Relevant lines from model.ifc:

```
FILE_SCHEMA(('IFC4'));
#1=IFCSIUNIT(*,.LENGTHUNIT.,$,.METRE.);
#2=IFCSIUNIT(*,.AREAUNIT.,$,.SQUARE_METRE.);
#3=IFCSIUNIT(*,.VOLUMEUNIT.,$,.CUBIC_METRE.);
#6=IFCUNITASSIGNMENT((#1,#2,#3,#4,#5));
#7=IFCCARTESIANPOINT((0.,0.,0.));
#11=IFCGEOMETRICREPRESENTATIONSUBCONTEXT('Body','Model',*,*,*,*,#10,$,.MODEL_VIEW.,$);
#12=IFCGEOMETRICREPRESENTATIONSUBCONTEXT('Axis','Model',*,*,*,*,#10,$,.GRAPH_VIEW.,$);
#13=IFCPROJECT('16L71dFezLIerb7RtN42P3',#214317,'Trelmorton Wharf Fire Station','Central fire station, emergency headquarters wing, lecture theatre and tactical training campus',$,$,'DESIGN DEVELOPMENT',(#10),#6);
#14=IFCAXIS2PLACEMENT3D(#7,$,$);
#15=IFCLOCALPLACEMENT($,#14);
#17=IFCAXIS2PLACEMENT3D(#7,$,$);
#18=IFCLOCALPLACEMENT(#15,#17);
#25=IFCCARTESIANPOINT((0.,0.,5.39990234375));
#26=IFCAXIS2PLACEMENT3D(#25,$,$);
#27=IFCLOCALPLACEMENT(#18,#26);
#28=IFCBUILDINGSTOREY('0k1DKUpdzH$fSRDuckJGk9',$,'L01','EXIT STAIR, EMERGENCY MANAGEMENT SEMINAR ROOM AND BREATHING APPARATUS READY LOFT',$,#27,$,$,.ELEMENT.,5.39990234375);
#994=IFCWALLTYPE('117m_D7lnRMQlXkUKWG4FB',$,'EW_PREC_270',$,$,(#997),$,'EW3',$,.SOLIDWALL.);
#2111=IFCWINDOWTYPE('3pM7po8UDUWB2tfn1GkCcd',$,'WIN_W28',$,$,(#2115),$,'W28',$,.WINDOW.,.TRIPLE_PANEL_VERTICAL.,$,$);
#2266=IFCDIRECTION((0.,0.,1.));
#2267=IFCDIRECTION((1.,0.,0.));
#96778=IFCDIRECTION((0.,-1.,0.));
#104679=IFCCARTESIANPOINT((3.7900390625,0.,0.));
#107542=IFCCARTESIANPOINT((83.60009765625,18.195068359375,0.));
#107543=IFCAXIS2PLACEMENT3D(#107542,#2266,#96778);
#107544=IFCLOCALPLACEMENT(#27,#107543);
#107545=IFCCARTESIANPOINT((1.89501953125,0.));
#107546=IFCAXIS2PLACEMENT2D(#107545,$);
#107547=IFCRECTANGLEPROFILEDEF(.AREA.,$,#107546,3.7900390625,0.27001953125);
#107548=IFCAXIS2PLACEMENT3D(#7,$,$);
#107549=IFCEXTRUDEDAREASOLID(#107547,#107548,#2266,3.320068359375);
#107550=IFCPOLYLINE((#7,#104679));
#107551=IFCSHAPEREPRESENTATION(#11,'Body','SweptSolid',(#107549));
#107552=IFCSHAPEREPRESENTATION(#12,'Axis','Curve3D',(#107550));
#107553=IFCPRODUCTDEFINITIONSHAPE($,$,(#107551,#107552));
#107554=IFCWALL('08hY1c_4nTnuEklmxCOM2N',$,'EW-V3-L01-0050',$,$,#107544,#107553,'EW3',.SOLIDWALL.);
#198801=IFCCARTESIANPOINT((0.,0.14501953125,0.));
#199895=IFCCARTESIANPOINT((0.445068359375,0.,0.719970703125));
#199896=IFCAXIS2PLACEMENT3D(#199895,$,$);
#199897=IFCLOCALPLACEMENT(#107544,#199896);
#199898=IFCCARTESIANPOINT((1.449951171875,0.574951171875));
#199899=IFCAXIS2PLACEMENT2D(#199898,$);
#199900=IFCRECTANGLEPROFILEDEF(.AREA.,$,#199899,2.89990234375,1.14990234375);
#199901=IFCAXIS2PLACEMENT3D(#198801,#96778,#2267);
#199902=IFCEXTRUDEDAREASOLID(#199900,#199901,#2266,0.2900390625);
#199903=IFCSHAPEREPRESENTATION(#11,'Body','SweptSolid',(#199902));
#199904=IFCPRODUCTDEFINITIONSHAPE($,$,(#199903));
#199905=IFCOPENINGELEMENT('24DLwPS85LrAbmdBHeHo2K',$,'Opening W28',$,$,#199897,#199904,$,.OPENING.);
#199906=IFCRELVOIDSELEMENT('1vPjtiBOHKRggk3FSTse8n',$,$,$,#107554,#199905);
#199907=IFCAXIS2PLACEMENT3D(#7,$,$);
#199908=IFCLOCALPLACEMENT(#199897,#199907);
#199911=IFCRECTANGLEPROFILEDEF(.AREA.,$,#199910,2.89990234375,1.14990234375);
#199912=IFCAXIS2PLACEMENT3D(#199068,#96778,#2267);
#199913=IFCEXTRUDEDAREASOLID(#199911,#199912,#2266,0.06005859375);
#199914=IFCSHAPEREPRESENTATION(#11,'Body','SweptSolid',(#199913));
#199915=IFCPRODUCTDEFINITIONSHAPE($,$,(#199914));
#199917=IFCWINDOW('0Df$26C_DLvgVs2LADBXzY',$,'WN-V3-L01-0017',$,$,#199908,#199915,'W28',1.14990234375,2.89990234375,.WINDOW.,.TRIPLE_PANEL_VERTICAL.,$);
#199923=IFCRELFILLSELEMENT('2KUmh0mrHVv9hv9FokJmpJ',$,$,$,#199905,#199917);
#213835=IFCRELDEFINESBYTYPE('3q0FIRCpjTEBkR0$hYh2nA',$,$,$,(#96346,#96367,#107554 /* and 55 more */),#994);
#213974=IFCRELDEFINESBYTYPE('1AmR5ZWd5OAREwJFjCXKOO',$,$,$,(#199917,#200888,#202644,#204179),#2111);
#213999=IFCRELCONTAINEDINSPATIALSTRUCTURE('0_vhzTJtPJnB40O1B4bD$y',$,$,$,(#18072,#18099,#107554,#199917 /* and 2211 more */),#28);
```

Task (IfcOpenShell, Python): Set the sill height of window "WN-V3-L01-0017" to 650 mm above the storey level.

```python
import numpy as np
import ifcopenshell
import ifcopenshell.api.geometry
import ifcopenshell.geom
import ifcopenshell.util.element
import ifcopenshell.util.placement
import ifcopenshell.util.shape
import ifcopenshell.util.unit

model = ifcopenshell.open("model.ifc")
unit_scale = ifcopenshell.util.unit.calculate_unit_scale(model)

window = model.by_guid("0Df$26C_DLvgVs2LADBXzY")
opening = window.FillsVoids[0].RelatingOpeningElement
storey = ifcopenshell.util.element.get_container(window, ifc_class="IfcBuildingStorey")
level = ifcopenshell.util.placement.get_local_placement(storey.ObjectPlacement)[2, 3]

# The opening's origin need not be at the sill, so measure its lowest point.
shape = ifcopenshell.geom.create_shape(ifcopenshell.geom.settings(), opening)
bottom = ifcopenshell.util.shape.get_shape_bottom_elevation(shape, shape.geometry) / unit_scale
dz = level + 0.65 - bottom

shift = np.array([0.0, 0.0, dz])
# The window is placed relative to its opening, so it follows when the opening moves.
matrix = ifcopenshell.util.placement.get_local_placement(opening.ObjectPlacement)
matrix[:3, 3] += shift
ifcopenshell.api.geometry.edit_object_placement(
    model, product=opening, matrix=matrix, is_si=False, should_transform_children=True
)

print(f"moved by {dz * unit_scale:+.3f} m")

model.write("model_v2.ifc")
```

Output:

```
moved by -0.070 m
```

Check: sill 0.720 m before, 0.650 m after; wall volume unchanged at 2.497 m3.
